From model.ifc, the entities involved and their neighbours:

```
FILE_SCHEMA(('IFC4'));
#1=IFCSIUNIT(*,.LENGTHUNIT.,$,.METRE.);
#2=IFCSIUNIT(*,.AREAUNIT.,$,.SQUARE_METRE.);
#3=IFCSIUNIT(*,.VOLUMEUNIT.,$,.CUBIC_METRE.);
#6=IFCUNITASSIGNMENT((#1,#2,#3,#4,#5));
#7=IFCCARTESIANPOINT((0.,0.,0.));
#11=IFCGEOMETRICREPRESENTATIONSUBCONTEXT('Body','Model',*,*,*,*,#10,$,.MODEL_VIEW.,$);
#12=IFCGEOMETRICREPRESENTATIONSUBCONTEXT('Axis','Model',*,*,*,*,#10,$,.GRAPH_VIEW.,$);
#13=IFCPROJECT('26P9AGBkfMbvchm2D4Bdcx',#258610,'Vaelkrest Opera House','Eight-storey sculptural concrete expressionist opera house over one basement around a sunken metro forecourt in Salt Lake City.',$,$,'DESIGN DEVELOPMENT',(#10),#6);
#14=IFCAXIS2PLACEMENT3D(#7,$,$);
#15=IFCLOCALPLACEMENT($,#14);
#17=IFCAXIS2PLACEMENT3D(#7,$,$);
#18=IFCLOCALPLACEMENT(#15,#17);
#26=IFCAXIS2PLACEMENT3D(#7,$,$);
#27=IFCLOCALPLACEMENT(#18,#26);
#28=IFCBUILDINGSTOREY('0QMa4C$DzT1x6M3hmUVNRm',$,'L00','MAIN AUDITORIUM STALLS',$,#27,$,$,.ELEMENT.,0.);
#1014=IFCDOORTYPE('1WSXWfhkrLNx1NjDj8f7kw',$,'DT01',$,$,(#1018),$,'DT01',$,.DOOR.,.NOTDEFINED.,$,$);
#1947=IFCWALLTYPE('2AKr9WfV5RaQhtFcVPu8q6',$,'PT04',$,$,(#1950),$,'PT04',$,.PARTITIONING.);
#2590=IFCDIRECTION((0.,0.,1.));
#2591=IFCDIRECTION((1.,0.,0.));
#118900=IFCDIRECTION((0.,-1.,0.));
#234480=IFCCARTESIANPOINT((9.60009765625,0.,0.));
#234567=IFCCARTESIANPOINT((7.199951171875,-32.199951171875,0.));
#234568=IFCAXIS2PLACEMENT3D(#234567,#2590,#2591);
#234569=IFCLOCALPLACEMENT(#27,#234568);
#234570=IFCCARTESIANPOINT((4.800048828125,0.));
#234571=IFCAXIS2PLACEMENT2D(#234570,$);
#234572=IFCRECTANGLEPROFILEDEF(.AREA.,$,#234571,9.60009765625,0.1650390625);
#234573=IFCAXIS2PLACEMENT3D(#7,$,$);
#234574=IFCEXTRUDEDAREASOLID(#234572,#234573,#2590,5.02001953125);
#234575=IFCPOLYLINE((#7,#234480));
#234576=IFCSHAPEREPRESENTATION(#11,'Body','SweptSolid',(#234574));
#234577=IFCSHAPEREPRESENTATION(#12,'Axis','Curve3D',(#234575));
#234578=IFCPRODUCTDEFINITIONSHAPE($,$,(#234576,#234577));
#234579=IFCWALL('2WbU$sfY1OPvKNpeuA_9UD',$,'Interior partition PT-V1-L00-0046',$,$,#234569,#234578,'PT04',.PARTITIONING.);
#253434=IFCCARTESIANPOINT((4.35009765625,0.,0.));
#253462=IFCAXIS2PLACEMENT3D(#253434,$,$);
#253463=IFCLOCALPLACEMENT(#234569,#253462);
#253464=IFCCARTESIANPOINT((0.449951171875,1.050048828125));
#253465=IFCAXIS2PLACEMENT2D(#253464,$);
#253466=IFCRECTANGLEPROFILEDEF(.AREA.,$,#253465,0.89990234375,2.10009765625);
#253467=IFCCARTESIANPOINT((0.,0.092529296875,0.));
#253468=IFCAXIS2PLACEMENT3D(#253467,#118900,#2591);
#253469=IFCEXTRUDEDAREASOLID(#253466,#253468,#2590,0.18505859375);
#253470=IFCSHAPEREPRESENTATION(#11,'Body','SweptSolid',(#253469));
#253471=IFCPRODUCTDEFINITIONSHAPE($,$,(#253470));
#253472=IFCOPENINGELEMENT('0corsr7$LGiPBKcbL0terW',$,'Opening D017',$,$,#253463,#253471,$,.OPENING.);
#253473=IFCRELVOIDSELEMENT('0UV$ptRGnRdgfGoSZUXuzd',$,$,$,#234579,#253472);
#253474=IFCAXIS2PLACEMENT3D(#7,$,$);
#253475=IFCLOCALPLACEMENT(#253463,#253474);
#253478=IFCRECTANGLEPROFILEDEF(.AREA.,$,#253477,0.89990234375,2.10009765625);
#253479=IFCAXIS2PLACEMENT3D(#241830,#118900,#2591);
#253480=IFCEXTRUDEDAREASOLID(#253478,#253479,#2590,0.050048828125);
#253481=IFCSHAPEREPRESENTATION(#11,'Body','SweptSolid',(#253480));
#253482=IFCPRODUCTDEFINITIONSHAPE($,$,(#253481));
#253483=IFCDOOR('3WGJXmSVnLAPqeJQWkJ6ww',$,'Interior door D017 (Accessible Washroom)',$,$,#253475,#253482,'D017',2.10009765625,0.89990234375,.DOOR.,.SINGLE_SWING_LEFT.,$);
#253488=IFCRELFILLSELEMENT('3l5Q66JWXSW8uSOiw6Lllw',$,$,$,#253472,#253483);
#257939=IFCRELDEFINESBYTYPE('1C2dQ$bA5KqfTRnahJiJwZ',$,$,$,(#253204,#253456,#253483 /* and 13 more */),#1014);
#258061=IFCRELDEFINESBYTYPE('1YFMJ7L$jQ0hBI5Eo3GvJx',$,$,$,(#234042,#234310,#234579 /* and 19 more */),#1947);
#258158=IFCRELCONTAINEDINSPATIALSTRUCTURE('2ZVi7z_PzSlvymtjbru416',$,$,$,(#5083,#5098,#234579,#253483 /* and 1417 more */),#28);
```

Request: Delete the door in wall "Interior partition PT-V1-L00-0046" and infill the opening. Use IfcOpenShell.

```python
import ifcopenshell
import ifcopenshell.api.feature
import ifcopenshell.api.root
import ifcopenshell.geom
import ifcopenshell.util.shape

model = ifcopenshell.open("model.ifc")
settings = ifcopenshell.geom.settings()


def volume(element):
    """Net volume in cubic metres, openings subtracted."""
    shape = ifcopenshell.geom.create_shape(settings, element)
    return ifcopenshell.util.shape.get_volume(shape.geometry)


door = model.by_guid("3WGJXmSVnLAPqeJQWkJ6ww")
opening = door.FillsVoids[0].RelatingOpeningElement
wall = opening.VoidsElements[0].RelatingBuildingElement
before = volume(wall)

ifcopenshell.api.root.remove_product(model, product=door)
ifcopenshell.api.feature.remove_feature(model, feature=opening)

after = volume(wall)

print(f"wall volume {before:.3f} -> {after:.3f} m3")

model.write("model-out.ifc")
```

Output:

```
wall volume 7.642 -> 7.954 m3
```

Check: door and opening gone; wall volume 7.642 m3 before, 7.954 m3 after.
